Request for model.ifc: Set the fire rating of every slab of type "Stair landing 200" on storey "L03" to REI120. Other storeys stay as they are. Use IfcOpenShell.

First a look at what the model holds.

```python
import ifcopenshell
import ifcopenshell.util.element

model = ifcopenshell.open("model.ifc")
print(model.schema)
storey = next(s for s in model.by_type("IfcBuildingStorey") if s.Name == "L03")
slabs = [e for e in ifcopenshell.util.element.get_decomposition(storey) if e.is_a("IfcSlab")]
seen = {}
for e in slabs:
    element_type = ifcopenshell.util.element.get_type(e)
    key = (element_type.Name if element_type != e and element_type else None, ifcopenshell.util.element.get_pset(e, "Pset_SlabCommon", "FireRating"))
    seen[key] = seen.get(key, 0) + 1
for (name, value), count in sorted(seen.items(), key=str):
    print(count, "x", name, "|", value)
```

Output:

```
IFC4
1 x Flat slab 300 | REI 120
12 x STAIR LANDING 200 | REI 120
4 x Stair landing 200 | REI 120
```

```python
import ifcopenshell
import ifcopenshell.api.pset
import ifcopenshell.util.element

model = ifcopenshell.open("model.ifc")

storey = next(s for s in model.by_type("IfcBuildingStorey") if s.Name == "L03")
slabs = [e for e in ifcopenshell.util.element.get_decomposition(storey) if e.is_a("IfcSlab")]

count = 0
for e in slabs:
    element_type = ifcopenshell.util.element.get_type(e)
    if element_type in (None, e) or element_type.Name != "Stair landing 200":
        continue
    found = ifcopenshell.util.element.get_pset(e, "Pset_SlabCommon", should_inherit=False)
    if found:
        pset = model.by_id(found["id"])
        if len(ifcopenshell.util.element.get_elements_by_pset(pset)) > 1:
            pset = ifcopenshell.api.pset.unshare_pset(model, products=[e], pset=pset)[0]
    else:
        pset = ifcopenshell.api.pset.add_pset(model, product=e, name="Pset_SlabCommon")
    ifcopenshell.api.pset.edit_pset(model, pset=pset, properties={"FireRating": "REI120"})
    count += 1

print(count, "slabs updated")

model.write("model_v2.ifc")
```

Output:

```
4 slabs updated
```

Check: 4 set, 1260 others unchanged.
